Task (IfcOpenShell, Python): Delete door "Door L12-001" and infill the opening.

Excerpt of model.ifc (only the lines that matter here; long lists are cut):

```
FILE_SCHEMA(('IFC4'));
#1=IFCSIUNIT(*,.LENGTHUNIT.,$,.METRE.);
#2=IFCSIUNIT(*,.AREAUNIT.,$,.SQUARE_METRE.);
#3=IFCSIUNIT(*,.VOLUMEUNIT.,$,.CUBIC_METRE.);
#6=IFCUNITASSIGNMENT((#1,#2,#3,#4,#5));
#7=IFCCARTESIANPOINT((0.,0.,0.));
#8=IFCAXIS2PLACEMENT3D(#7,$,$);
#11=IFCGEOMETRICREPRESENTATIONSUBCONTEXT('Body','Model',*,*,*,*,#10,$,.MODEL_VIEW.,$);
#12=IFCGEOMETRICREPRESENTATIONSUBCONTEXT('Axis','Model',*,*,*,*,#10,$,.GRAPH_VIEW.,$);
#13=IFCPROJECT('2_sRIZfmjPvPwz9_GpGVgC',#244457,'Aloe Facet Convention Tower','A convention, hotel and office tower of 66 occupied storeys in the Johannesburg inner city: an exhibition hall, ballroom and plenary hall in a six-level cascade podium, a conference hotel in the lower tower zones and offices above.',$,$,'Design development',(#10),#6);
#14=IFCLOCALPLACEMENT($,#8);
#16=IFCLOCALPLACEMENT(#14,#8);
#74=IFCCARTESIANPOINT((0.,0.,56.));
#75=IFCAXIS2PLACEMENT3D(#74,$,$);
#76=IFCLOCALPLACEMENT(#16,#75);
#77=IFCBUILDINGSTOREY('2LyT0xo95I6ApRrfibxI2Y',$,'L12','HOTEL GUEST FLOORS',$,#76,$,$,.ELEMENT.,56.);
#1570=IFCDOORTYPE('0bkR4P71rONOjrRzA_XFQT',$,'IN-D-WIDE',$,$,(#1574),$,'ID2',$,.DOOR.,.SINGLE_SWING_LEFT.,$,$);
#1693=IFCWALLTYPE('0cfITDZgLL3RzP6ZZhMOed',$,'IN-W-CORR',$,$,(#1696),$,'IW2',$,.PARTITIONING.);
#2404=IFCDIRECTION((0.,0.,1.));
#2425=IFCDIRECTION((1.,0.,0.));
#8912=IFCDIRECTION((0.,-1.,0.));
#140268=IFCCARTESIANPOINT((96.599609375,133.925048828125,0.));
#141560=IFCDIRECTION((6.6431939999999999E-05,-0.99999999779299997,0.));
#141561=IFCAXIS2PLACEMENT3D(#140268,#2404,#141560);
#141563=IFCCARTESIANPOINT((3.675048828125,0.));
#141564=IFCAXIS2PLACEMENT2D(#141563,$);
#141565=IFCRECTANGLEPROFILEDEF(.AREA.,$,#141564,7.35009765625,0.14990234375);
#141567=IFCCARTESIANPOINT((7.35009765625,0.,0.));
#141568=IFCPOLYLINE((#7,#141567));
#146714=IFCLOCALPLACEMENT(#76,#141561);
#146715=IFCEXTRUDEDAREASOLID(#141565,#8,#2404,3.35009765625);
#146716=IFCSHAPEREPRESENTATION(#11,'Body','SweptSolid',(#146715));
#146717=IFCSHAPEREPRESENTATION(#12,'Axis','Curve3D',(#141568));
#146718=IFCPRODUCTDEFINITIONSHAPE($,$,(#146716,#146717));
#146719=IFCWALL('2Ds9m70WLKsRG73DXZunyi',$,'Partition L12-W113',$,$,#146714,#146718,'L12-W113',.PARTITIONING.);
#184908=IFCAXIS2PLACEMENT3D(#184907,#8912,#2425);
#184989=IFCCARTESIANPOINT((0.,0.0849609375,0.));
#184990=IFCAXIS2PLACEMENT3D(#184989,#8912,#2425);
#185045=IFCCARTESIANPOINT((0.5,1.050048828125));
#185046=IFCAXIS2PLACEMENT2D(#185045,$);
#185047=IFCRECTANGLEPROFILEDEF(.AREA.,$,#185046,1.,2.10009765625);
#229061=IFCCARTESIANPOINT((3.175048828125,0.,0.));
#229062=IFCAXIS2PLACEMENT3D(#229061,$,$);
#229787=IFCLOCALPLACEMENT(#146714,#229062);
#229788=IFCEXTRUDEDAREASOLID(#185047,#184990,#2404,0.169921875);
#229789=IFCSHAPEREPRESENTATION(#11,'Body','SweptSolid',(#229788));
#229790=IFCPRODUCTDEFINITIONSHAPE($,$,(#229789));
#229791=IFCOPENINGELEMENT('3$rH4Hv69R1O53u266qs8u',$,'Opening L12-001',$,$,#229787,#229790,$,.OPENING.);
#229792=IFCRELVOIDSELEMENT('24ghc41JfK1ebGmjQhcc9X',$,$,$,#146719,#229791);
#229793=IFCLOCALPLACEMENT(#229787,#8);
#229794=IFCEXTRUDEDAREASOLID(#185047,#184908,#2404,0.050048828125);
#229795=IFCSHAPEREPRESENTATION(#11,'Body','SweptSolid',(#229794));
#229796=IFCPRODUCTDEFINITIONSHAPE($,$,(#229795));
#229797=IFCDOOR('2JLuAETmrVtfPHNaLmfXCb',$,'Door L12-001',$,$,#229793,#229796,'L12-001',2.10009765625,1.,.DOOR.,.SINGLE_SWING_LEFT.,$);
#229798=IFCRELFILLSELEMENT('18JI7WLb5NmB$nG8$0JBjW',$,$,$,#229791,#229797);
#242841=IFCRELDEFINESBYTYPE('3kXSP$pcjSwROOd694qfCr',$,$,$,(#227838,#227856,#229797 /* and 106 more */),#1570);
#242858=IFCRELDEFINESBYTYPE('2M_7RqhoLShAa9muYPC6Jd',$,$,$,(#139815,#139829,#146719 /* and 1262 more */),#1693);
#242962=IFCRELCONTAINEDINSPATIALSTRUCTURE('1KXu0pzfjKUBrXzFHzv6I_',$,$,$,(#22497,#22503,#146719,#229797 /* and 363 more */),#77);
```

```python
import ifcopenshell
import ifcopenshell.api.feature
import ifcopenshell.api.root
import ifcopenshell.geom
import ifcopenshell.util.shape

model = ifcopenshell.open("model.ifc")
settings = ifcopenshell.geom.settings()


def volume(element):
    """Net volume in cubic metres, openings subtracted."""
    shape = ifcopenshell.geom.create_shape(settings, element)
    return ifcopenshell.util.shape.get_volume(shape.geometry)


door = model.by_guid("2JLuAETmrVtfPHNaLmfXCb")
opening = door.FillsVoids[0].RelatingOpeningElement
wall = opening.VoidsElements[0].RelatingBuildingElement
before = volume(wall)

ifcopenshell.api.root.remove_product(model, product=door)
ifcopenshell.api.feature.remove_feature(model, feature=opening)

after = volume(wall)

print(f"wall volume {before:.3f} -> {after:.3f} m3")

model.write("model_updated.ifc")
```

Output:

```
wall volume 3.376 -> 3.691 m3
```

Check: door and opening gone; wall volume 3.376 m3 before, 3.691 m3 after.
